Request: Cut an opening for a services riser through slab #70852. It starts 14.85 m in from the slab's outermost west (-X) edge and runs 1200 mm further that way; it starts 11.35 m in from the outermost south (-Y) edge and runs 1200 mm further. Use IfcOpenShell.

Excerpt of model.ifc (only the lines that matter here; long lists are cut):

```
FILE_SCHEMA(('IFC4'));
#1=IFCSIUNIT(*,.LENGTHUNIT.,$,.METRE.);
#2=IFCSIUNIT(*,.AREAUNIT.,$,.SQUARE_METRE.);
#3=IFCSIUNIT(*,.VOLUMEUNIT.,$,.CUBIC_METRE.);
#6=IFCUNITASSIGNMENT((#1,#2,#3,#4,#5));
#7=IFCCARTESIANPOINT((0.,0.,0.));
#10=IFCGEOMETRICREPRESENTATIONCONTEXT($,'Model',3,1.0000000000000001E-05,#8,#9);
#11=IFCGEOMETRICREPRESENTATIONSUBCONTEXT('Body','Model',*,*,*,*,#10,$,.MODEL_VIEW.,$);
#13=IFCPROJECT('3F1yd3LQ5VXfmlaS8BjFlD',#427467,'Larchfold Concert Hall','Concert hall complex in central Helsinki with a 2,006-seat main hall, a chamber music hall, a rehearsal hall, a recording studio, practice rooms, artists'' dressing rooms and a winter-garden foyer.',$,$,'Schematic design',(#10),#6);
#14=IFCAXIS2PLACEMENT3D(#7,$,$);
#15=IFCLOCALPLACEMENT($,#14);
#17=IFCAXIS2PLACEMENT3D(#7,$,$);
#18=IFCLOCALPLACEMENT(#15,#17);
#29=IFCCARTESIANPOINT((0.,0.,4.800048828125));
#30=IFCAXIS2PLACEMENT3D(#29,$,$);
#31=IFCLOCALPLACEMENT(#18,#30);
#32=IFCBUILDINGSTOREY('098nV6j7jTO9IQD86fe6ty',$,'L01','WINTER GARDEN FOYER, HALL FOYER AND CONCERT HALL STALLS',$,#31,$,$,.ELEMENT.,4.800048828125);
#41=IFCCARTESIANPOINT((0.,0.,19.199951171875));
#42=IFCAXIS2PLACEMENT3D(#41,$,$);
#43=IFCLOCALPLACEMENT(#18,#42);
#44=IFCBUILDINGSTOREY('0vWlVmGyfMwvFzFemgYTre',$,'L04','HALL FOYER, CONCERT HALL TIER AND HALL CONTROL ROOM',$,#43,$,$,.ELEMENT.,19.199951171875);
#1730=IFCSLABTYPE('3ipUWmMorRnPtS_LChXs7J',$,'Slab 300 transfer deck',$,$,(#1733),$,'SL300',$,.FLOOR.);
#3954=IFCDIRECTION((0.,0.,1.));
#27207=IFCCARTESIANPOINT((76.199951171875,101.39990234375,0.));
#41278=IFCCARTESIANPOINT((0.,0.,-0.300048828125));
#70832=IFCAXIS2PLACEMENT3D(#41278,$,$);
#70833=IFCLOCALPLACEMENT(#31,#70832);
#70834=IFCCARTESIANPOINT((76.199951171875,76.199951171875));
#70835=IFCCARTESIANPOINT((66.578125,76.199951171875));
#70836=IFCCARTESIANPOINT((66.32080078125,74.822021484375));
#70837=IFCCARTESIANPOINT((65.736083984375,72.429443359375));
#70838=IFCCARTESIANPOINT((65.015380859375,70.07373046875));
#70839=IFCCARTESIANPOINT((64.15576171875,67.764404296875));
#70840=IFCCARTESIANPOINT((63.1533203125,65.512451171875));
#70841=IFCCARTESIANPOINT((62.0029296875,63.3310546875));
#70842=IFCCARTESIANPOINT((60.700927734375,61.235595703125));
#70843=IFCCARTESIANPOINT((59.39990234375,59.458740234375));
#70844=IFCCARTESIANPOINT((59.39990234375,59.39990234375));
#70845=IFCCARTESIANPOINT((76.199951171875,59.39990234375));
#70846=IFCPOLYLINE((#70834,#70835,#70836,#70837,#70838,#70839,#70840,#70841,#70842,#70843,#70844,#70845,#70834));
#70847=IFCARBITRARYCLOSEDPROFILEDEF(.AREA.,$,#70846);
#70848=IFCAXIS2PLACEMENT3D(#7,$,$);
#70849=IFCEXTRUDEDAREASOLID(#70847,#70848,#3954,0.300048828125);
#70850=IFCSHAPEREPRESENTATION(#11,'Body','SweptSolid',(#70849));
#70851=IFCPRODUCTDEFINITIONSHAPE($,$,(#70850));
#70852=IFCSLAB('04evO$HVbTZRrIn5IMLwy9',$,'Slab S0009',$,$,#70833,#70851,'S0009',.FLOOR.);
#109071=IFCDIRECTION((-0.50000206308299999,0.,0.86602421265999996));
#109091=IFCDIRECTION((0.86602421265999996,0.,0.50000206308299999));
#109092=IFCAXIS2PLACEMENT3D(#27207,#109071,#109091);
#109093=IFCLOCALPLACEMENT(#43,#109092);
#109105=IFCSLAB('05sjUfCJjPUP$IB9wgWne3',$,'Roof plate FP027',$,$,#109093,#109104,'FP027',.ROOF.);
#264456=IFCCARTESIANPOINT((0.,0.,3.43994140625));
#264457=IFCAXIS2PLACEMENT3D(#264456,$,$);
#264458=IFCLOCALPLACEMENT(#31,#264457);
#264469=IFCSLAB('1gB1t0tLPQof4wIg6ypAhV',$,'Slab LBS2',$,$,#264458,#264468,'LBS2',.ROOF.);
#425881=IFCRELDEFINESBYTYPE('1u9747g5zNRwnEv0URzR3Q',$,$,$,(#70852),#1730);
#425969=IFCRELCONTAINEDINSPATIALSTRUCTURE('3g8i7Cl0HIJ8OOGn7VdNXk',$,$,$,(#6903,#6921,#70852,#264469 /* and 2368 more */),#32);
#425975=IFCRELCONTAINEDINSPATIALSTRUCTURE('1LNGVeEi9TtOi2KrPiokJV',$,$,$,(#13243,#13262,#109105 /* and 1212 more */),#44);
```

```python
import numpy as np
import ifcopenshell
import ifcopenshell.api.feature
import ifcopenshell.api.geometry
import ifcopenshell.api.root
import ifcopenshell.geom
import ifcopenshell.util.placement
import ifcopenshell.util.representation
import ifcopenshell.util.shape
import ifcopenshell.util.unit

model = ifcopenshell.open("model.ifc")
unit_scale = ifcopenshell.util.unit.calculate_unit_scale(model)
settings = ifcopenshell.geom.settings()


def volume(element):
    """Net volume in cubic metres, openings subtracted."""
    shape = ifcopenshell.geom.create_shape(settings, element)
    return ifcopenshell.util.shape.get_volume(shape.geometry)


slab = model.by_guid("04evO$HVbTZRrIn5IMLwy9")
before = volume(slab)

# Extent in the slab's own axes, in metres. The edges named are its -X and -Y sides.
slab_shape = ifcopenshell.geom.create_shape(settings, slab)
vertices = ifcopenshell.util.shape.get_vertices(slab_shape.geometry)
x_min, y_min, bottom = vertices.min(axis=0)
top = vertices[:, 2].max()

opening = ifcopenshell.api.root.create_entity(model, ifc_class="IfcOpeningElement", name="Services riser opening", predefined_type="OPENING")
context = ifcopenshell.util.representation.get_context(model, "Model", "Body", "MODEL_VIEW")
width, depth = 1.2, 1.2
outline = [(0.0, 0.0), (width, 0.0), (width, depth), (0.0, depth), (0.0, 0.0)]
# Overshoot both faces by 50 mm so the cut is clean.
shape = ifcopenshell.api.geometry.add_slab_representation(
    model, context=context, depth=top - bottom + 0.1, polyline=outline
)
ifcopenshell.api.geometry.assign_representation(model, product=opening, representation=shape)

matrix = ifcopenshell.util.placement.get_local_placement(slab.ObjectPlacement)
matrix[:, 3] = matrix @ np.append(np.array([x_min + 14.85, y_min + 11.35, bottom - 0.05]) / unit_scale, 1.0)
ifcopenshell.api.geometry.edit_object_placement(model, product=opening, matrix=matrix, is_si=False)
ifcopenshell.api.feature.add_feature(model, feature=opening, element=slab)

after = volume(slab)

print(f"slab volume {before:.3f} -> {after:.3f} m3")

model.write("model_v2.ifc")
```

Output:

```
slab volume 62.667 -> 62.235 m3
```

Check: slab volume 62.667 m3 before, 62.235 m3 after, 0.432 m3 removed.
